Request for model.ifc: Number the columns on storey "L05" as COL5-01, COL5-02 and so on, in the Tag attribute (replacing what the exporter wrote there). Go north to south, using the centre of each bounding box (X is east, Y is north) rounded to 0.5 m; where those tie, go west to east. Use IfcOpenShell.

First a look at what the model holds.

```python
import ifcopenshell
import ifcopenshell.util.element
import ifcopenshell.util.placement

model = ifcopenshell.open("model.ifc")
print(model.schema)
storey = next(s for s in model.by_type("IfcBuildingStorey") if s.Name == "L05")
columns = [e for e in ifcopenshell.util.element.get_decomposition(storey) if e.is_a("IfcColumn")]
for e in sorted(columns, key=lambda e: e.id()):
    origin = ifcopenshell.util.placement.get_local_placement(e.ObjectPlacement)[:3, 3]
    print(e.id(), e.Tag, e.Name, origin.round(2) + 0.0, sep=" | ")
```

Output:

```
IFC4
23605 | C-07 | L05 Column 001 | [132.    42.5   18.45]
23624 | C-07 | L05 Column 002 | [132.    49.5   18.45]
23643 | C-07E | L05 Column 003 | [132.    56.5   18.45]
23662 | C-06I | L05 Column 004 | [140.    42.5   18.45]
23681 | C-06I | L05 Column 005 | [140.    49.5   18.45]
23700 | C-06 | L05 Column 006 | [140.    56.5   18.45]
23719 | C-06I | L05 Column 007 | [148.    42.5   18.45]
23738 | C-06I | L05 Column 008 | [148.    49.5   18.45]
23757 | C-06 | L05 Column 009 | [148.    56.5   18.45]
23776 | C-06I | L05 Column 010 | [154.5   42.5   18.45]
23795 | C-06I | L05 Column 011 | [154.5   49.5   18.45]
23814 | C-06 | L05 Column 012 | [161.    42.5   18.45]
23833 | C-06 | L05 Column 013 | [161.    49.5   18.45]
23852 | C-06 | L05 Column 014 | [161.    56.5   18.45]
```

```python
import ifcopenshell
import ifcopenshell.geom
import ifcopenshell.util.element
import ifcopenshell.util.shape

model = ifcopenshell.open("model.ifc")
settings = ifcopenshell.geom.settings()
settings.set("use-world-coords", True)


def centre(element):
    shape = ifcopenshell.geom.create_shape(settings, element)
    return ifcopenshell.util.shape.get_bbox_centroid(shape.geometry)


storey = next(s for s in model.by_type("IfcBuildingStorey") if s.Name == "L05")
columns = [e for e in ifcopenshell.util.element.get_decomposition(storey) if e.is_a("IfcColumn")]

# Insertion points can sit at a corner or the storey origin, so sort by the geometry (in metres).
centres = {e: centre(e) for e in columns}
columns.sort(key=lambda e: (-round(centres[e][1] / 0.5), centres[e][0]))

for i, e in enumerate(columns, start=1):
    number = f"COL5-{i:02d}"
    e.Tag = number
    print(e.id(), number)

model.write("model_rev.ifc")
```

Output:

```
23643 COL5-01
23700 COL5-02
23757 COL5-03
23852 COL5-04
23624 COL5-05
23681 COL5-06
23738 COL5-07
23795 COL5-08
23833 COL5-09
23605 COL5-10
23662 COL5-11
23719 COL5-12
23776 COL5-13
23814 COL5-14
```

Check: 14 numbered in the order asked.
